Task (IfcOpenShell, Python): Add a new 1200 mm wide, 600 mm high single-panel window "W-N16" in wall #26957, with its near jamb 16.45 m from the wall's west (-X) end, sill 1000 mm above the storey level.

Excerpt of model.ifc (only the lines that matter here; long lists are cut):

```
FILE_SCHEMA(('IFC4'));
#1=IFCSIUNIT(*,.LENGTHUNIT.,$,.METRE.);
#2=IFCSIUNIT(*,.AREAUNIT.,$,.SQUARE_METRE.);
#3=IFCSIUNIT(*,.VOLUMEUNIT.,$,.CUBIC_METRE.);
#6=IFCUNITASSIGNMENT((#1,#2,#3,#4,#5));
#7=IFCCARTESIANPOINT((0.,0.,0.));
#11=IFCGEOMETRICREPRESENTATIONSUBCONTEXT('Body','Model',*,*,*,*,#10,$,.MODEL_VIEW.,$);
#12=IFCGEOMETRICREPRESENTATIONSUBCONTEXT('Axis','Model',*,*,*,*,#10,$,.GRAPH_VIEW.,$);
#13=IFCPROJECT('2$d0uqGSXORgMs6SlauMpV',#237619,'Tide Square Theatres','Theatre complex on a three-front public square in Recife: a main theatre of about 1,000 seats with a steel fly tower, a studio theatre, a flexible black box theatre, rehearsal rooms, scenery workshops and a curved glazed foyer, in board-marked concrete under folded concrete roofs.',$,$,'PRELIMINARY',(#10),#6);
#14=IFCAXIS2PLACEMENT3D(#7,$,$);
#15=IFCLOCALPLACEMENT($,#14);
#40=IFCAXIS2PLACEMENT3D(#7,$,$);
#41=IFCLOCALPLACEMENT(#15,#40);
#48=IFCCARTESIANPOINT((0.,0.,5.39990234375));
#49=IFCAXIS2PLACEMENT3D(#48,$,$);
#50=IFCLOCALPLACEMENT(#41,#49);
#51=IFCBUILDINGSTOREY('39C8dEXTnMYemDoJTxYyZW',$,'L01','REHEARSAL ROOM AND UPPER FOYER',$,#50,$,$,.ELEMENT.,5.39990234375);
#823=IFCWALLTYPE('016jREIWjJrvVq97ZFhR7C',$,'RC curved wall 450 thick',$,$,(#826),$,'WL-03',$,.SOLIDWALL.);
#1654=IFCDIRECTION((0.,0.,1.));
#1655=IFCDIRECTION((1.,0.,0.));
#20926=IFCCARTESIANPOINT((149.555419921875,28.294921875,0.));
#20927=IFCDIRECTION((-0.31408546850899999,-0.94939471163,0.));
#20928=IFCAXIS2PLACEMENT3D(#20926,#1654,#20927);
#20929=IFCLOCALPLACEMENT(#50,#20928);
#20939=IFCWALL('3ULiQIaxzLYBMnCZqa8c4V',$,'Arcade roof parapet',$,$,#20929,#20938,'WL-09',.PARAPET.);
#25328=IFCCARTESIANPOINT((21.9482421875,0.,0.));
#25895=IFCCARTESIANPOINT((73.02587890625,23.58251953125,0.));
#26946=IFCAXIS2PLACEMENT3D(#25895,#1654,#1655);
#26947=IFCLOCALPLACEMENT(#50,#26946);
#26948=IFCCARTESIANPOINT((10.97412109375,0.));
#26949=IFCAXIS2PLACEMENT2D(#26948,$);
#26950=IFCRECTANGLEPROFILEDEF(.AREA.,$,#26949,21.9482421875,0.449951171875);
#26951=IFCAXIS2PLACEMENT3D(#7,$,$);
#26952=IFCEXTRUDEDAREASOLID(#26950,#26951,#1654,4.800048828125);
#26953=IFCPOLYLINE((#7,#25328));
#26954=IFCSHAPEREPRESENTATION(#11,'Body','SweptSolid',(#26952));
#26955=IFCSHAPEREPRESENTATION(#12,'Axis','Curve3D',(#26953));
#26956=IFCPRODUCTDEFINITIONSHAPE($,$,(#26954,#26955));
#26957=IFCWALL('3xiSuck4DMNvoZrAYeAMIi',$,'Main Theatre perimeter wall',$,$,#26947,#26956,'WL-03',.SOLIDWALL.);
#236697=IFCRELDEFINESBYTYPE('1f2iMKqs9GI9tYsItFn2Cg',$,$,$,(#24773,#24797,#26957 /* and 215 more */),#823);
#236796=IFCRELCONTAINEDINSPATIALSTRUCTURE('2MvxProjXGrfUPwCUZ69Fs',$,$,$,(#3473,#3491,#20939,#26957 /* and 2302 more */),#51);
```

```python
import numpy as np
import ifcopenshell
import ifcopenshell.api.feature
import ifcopenshell.api.geometry
import ifcopenshell.api.root
import ifcopenshell.api.spatial
import ifcopenshell.geom
import ifcopenshell.util.element
import ifcopenshell.util.placement
import ifcopenshell.util.representation
import ifcopenshell.util.shape
import ifcopenshell.util.unit

model = ifcopenshell.open("model.ifc")
unit_scale = ifcopenshell.util.unit.calculate_unit_scale(model)
settings = ifcopenshell.geom.settings()


def volume(element):
    """Net volume in cubic metres, openings subtracted."""
    shape = ifcopenshell.geom.create_shape(settings, element)
    return ifcopenshell.util.shape.get_volume(shape.geometry)


wall = model.by_id(26957)
storey = ifcopenshell.util.element.get_container(wall, ifc_class="IfcBuildingStorey")
context = ifcopenshell.util.representation.get_context(model, "Model", "Body", "MODEL_VIEW")
before = volume(wall)

width, height, from_end, sill = 1.2, 0.6, 16.45, 1  # metres

# The wall runs along its own X axis, and the end named is its -X end.
wall_shape = ifcopenshell.geom.create_shape(settings, wall)
x, y, z = ifcopenshell.util.shape.get_vertices(wall_shape.geometry).T
start = x.min() + from_end
face, thickness = float(y.min()), float(y.max() - y.min())
wall_matrix = ifcopenshell.util.placement.get_local_placement(wall.ObjectPlacement)
level = ifcopenshell.util.placement.get_local_placement(storey.ObjectPlacement)[2, 3]


def in_wall(x, y):
    """Placement at x, y metres in the wall's axes, at sill height."""
    matrix = wall_matrix.copy()
    matrix[:, 3] = wall_matrix @ np.array([x / unit_scale, y / unit_scale, 0.0, 1.0])
    matrix[2, 3] = level + sill / unit_scale
    return matrix


# Opening: a box that overshoots both wall faces by 50 mm.
opening = ifcopenshell.api.root.create_entity(model, ifc_class="IfcOpeningElement", predefined_type="OPENING")
box = ifcopenshell.api.geometry.add_wall_representation(
    model, context=context, length=width, height=height, thickness=thickness + 0.1
)
ifcopenshell.api.geometry.assign_representation(model, product=opening, representation=box)
ifcopenshell.api.geometry.edit_object_placement(model, product=opening, matrix=in_wall(start, face - 0.05), is_si=False)
ifcopenshell.api.feature.add_feature(model, feature=opening, element=wall)

window = ifcopenshell.api.root.create_entity(model, ifc_class="IfcWindow", name="W-N16", predefined_type="WINDOW")
window.OverallWidth, window.OverallHeight = width / unit_scale, height / unit_scale
window.PartitioningType = "SINGLE_PANEL"
body = ifcopenshell.api.geometry.add_window_representation(
    model,
    context=context,
    overall_width=window.OverallWidth,
    overall_height=window.OverallHeight,
    partition_type="SINGLE_PANEL",
)
ifcopenshell.api.geometry.assign_representation(model, product=window, representation=body)
ifcopenshell.api.spatial.assign_container(model, products=[window], relating_structure=storey)
ifcopenshell.api.feature.add_filling(model, opening=opening, element=window)

# Centre the window in the wall's thickness.
ifcopenshell.api.geometry.edit_object_placement(model, product=window, matrix=in_wall(start, face), is_si=False)
window_shape = ifcopenshell.geom.create_shape(settings, window)
depth = ifcopenshell.util.shape.get_vertices(window_shape.geometry)[:, 1]
offset = face + thickness / 2 - (depth.min() + depth.max()) / 2
ifcopenshell.api.geometry.edit_object_placement(model, product=window, matrix=in_wall(start, offset), is_si=False)

after = volume(wall)

print(f"wall volume {before:.3f} -> {after:.3f} m3")

model.write("model_v2.ifc")
```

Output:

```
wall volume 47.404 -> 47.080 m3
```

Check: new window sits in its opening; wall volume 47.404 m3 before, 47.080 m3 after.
